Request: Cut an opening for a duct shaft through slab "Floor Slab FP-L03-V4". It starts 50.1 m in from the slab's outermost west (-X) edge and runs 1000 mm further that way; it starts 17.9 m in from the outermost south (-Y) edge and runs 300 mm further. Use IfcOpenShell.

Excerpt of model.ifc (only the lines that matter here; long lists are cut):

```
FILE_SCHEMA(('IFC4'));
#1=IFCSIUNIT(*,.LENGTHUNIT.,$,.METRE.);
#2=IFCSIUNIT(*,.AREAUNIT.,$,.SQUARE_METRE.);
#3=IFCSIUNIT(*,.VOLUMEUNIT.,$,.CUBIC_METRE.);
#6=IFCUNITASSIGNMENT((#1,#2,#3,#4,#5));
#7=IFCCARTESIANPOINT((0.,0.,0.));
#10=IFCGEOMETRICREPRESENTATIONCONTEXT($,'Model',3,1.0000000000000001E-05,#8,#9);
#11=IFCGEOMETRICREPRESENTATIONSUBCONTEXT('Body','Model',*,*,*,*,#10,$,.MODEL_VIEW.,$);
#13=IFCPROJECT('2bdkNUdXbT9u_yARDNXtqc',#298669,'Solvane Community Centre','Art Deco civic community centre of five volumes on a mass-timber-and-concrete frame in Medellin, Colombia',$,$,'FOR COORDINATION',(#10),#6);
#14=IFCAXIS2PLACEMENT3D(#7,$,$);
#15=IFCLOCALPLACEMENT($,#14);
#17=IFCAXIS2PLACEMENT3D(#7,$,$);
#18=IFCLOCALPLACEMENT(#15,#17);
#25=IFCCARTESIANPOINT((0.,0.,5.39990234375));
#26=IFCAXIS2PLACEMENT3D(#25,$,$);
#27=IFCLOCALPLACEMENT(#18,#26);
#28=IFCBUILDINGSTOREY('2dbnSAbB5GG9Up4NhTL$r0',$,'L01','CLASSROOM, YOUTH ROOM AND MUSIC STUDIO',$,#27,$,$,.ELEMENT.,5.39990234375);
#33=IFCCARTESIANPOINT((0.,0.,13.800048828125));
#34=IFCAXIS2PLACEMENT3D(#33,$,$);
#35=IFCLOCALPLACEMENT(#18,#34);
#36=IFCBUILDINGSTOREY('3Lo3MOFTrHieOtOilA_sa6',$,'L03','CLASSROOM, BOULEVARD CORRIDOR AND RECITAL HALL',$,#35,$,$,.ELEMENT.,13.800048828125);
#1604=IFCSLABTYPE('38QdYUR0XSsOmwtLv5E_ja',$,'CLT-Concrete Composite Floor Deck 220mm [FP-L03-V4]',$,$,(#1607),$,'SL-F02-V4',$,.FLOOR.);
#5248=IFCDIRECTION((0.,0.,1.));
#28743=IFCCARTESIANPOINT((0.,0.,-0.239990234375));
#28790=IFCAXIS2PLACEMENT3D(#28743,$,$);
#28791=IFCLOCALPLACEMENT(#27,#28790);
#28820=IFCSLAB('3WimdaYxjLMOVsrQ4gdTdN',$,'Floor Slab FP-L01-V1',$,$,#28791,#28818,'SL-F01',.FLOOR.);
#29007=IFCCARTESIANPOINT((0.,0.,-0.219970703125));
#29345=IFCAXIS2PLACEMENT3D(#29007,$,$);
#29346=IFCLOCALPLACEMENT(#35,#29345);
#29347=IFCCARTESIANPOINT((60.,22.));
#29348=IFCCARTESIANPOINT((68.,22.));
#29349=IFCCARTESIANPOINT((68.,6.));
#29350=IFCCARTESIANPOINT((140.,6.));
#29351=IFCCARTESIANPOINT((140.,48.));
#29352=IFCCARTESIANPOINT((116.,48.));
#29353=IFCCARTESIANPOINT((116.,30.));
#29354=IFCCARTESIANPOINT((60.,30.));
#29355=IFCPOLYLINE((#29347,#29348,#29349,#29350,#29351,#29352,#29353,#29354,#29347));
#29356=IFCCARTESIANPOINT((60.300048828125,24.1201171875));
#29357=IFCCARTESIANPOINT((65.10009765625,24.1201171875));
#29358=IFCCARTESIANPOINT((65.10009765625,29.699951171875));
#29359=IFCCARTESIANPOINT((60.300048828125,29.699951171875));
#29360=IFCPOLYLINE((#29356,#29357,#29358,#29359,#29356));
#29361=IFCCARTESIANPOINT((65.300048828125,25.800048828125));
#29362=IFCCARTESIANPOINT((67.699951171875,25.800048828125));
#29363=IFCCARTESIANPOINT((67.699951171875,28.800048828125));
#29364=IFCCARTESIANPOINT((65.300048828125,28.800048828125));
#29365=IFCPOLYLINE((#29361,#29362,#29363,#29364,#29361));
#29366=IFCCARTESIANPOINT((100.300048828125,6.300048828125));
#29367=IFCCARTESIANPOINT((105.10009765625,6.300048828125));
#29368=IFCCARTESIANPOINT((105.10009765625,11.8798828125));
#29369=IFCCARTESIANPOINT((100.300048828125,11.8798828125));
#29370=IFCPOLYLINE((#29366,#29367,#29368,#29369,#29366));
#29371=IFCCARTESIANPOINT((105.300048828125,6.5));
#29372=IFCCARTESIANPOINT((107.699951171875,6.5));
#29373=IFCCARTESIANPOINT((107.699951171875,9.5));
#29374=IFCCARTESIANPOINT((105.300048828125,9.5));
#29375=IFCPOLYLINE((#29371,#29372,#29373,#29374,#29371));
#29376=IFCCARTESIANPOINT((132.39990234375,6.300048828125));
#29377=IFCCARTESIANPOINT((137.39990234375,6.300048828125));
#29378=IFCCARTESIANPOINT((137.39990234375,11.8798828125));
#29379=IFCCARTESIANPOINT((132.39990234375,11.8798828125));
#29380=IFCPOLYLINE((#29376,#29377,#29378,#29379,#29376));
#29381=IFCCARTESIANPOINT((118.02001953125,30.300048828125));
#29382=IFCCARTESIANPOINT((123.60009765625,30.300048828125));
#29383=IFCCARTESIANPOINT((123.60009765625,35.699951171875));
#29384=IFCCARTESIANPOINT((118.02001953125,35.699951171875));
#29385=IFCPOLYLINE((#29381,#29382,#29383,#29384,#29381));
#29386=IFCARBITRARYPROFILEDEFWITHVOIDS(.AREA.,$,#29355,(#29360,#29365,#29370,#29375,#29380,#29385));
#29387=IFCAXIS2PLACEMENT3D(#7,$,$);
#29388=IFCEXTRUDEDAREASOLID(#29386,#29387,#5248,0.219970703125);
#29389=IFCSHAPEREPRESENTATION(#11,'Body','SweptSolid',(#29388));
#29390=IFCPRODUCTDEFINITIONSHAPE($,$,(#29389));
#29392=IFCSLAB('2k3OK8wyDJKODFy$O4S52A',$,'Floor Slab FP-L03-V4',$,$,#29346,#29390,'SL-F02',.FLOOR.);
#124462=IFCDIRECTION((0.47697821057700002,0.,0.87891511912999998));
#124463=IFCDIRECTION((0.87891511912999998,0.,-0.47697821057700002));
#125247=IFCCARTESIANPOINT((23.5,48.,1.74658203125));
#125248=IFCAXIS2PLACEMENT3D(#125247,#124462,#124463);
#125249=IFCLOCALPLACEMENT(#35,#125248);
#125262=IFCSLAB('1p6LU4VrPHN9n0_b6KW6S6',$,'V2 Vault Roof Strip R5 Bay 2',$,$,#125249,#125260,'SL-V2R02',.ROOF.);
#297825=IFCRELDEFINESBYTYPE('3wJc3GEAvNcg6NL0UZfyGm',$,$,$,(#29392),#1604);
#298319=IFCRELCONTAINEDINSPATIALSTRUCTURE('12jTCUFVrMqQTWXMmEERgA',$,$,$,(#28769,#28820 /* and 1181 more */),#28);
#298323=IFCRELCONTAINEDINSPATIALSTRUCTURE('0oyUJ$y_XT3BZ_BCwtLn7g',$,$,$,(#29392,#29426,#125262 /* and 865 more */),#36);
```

```python
import numpy as np
import ifcopenshell
import ifcopenshell.api.feature
import ifcopenshell.api.geometry
import ifcopenshell.api.root
import ifcopenshell.geom
import ifcopenshell.util.placement
import ifcopenshell.util.representation
import ifcopenshell.util.shape
import ifcopenshell.util.unit

model = ifcopenshell.open("model.ifc")
unit_scale = ifcopenshell.util.unit.calculate_unit_scale(model)
settings = ifcopenshell.geom.settings()


def volume(element):
    """Net volume in cubic metres, openings subtracted."""
    shape = ifcopenshell.geom.create_shape(settings, element)
    return ifcopenshell.util.shape.get_volume(shape.geometry)


slab = model.by_guid("2k3OK8wyDJKODFy$O4S52A")
before = volume(slab)

# Extent in the slab's own axes, in metres. The edges named are its -X and -Y sides.
slab_shape = ifcopenshell.geom.create_shape(settings, slab)
vertices = ifcopenshell.util.shape.get_vertices(slab_shape.geometry)
x_min, y_min, bottom = vertices.min(axis=0)
top = vertices[:, 2].max()

opening = ifcopenshell.api.root.create_entity(model, ifc_class="IfcOpeningElement", name="Duct shaft opening", predefined_type="OPENING")
context = ifcopenshell.util.representation.get_context(model, "Model", "Body", "MODEL_VIEW")
width, depth = 1, 0.3
outline = [(0.0, 0.0), (width, 0.0), (width, depth), (0.0, depth), (0.0, 0.0)]
# Overshoot both faces by 50 mm so the cut is clean.
shape = ifcopenshell.api.geometry.add_slab_representation(
    model, context=context, depth=top - bottom + 0.1, polyline=outline
)
ifcopenshell.api.geometry.assign_representation(model, product=opening, representation=shape)

matrix = ifcopenshell.util.placement.get_local_placement(slab.ObjectPlacement)
matrix[:, 3] = matrix @ np.append(np.array([x_min + 50.1, y_min + 17.9, bottom - 0.05]) / unit_scale, 1.0)
ifcopenshell.api.geometry.edit_object_placement(model, product=opening, matrix=matrix, is_si=False)
ifcopenshell.api.feature.add_feature(model, feature=opening, element=slab)

after = volume(slab)

print(f"slab volume {before:.3f} -> {after:.3f} m3")

model.write("model_v2.ifc")
```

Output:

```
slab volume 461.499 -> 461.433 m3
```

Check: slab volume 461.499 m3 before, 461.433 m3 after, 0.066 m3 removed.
